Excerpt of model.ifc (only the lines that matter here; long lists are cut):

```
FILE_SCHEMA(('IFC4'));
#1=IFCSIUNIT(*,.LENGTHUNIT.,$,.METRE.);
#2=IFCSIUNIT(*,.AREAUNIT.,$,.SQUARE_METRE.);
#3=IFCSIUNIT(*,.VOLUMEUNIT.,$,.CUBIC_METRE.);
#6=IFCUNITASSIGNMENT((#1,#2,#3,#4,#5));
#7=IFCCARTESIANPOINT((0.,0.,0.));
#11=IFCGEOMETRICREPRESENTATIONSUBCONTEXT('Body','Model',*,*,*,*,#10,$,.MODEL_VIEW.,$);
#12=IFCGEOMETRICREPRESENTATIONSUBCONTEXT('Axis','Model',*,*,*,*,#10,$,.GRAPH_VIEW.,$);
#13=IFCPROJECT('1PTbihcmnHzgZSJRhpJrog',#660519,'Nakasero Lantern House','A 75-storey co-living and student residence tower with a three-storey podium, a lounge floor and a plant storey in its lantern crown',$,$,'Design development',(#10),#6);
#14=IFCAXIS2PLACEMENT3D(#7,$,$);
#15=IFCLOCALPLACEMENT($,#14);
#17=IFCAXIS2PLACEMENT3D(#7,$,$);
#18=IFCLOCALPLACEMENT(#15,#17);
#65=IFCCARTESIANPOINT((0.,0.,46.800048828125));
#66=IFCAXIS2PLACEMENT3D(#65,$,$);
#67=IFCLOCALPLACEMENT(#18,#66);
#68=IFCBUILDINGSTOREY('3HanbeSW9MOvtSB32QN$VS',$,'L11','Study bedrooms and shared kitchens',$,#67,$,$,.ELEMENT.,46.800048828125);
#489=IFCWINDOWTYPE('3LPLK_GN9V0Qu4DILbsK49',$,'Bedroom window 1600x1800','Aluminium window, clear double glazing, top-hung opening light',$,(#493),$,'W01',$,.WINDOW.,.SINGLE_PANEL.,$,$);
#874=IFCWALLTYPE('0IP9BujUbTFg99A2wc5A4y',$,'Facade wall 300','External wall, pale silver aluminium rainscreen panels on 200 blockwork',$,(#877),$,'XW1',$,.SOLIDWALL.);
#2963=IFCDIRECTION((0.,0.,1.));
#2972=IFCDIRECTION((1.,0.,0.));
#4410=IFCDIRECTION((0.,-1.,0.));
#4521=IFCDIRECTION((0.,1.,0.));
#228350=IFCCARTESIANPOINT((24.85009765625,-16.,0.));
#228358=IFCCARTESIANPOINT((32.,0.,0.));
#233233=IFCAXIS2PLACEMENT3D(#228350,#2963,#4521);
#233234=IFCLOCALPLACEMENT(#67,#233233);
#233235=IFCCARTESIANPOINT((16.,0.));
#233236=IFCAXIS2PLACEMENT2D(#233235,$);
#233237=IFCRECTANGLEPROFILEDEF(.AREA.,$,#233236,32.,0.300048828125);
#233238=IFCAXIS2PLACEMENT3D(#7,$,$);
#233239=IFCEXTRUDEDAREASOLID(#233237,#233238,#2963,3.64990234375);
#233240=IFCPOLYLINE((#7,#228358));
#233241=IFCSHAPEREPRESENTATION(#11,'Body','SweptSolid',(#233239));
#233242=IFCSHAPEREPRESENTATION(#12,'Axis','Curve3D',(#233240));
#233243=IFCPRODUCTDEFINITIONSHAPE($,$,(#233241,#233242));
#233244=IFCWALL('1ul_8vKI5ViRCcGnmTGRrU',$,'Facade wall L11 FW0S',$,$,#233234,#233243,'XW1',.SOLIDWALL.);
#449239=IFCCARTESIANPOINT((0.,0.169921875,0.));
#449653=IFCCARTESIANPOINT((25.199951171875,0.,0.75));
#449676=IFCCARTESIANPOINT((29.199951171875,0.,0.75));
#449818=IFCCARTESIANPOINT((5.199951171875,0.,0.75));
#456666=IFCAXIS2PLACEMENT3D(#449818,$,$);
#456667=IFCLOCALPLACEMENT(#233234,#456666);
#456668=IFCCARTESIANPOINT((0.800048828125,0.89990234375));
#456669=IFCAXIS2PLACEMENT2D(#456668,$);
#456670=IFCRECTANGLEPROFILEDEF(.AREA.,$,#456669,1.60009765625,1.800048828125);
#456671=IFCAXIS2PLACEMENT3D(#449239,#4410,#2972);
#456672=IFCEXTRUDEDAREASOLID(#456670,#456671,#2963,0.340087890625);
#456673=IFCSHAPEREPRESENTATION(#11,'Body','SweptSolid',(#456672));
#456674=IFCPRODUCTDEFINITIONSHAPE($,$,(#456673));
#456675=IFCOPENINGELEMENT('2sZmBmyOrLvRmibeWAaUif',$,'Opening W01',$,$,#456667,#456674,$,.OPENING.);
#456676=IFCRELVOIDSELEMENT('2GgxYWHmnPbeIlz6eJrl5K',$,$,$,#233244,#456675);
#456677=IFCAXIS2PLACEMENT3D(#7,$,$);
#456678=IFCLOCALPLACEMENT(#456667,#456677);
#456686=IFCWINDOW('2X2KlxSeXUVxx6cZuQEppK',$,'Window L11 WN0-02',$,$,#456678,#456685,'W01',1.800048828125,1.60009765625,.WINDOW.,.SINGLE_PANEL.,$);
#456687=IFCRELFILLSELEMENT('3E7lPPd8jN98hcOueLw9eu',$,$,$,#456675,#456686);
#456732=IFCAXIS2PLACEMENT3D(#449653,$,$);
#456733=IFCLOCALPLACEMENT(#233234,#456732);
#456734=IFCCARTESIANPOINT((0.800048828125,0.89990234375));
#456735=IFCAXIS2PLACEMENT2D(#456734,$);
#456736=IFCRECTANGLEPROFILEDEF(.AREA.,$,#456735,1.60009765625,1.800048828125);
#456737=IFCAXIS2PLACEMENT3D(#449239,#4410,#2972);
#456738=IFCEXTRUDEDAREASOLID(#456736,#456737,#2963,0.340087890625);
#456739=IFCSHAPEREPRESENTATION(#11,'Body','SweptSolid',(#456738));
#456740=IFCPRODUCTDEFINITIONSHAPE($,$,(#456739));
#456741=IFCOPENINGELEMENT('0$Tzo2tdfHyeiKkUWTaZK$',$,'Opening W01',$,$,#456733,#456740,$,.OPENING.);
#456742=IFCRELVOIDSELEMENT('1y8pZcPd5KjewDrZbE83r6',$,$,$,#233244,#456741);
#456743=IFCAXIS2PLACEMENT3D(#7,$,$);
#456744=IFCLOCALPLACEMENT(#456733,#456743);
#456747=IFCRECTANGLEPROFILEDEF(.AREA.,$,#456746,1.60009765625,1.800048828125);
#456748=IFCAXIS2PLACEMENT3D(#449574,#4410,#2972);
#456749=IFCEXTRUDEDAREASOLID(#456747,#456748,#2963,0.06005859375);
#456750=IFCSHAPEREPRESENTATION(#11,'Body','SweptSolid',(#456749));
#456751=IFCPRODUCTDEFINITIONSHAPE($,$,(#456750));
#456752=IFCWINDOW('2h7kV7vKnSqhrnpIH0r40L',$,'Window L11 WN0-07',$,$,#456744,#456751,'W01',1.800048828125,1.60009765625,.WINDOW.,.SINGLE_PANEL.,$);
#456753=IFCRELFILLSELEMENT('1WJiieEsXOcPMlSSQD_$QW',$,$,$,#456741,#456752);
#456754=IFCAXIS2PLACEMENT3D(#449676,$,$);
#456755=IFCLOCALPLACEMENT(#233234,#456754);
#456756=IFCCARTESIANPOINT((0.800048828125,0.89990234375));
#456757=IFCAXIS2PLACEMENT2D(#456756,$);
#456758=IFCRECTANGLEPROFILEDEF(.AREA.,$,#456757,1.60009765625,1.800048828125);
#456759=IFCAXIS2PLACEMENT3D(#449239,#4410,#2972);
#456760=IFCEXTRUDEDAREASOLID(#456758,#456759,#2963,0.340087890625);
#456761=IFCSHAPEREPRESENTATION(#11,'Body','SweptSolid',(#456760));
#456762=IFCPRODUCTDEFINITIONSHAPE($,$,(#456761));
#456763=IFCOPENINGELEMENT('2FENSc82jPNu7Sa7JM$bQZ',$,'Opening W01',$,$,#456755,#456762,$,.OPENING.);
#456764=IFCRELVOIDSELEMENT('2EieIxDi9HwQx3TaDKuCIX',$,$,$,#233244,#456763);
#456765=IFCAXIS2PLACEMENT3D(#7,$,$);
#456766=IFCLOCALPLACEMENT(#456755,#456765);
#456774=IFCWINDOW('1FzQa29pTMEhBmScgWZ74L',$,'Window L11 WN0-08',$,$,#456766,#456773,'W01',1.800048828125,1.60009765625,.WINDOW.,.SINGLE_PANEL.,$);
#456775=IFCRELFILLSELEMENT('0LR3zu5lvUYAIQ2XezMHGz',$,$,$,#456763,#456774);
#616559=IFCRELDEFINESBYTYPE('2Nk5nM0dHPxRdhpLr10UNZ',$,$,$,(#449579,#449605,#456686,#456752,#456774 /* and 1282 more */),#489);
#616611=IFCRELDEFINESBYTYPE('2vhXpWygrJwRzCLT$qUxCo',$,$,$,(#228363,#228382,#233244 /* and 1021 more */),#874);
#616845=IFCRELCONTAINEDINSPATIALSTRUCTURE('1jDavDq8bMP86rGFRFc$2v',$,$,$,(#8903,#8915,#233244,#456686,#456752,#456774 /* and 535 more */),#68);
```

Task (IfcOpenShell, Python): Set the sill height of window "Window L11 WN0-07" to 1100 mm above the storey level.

```python
import numpy as np
import ifcopenshell
import ifcopenshell.api.geometry
import ifcopenshell.geom
import ifcopenshell.util.element
import ifcopenshell.util.placement
import ifcopenshell.util.shape
import ifcopenshell.util.unit

model = ifcopenshell.open("model.ifc")
unit_scale = ifcopenshell.util.unit.calculate_unit_scale(model)

window = model.by_id(456752)
opening = window.FillsVoids[0].RelatingOpeningElement
storey = ifcopenshell.util.element.get_container(window, ifc_class="IfcBuildingStorey")
level = ifcopenshell.util.placement.get_local_placement(storey.ObjectPlacement)[2, 3]

# The opening's origin need not be at the sill, so measure its lowest point.
shape = ifcopenshell.geom.create_shape(ifcopenshell.geom.settings(), opening)
bottom = ifcopenshell.util.shape.get_shape_bottom_elevation(shape, shape.geometry) / unit_scale
dz = level + 1.1 - bottom

shift = np.array([0.0, 0.0, dz])
# The window is placed relative to its opening, so it follows when the opening moves.
matrix = ifcopenshell.util.placement.get_local_placement(opening.ObjectPlacement)
matrix[:3, 3] += shift
ifcopenshell.api.geometry.edit_object_placement(
    model, product=opening, matrix=matrix, is_si=False, should_transform_children=True
)

print(f"moved by {dz * unit_scale:+.3f} m")

model.write("model_rev.ifc")
```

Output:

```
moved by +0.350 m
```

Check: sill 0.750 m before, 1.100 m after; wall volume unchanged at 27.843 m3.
